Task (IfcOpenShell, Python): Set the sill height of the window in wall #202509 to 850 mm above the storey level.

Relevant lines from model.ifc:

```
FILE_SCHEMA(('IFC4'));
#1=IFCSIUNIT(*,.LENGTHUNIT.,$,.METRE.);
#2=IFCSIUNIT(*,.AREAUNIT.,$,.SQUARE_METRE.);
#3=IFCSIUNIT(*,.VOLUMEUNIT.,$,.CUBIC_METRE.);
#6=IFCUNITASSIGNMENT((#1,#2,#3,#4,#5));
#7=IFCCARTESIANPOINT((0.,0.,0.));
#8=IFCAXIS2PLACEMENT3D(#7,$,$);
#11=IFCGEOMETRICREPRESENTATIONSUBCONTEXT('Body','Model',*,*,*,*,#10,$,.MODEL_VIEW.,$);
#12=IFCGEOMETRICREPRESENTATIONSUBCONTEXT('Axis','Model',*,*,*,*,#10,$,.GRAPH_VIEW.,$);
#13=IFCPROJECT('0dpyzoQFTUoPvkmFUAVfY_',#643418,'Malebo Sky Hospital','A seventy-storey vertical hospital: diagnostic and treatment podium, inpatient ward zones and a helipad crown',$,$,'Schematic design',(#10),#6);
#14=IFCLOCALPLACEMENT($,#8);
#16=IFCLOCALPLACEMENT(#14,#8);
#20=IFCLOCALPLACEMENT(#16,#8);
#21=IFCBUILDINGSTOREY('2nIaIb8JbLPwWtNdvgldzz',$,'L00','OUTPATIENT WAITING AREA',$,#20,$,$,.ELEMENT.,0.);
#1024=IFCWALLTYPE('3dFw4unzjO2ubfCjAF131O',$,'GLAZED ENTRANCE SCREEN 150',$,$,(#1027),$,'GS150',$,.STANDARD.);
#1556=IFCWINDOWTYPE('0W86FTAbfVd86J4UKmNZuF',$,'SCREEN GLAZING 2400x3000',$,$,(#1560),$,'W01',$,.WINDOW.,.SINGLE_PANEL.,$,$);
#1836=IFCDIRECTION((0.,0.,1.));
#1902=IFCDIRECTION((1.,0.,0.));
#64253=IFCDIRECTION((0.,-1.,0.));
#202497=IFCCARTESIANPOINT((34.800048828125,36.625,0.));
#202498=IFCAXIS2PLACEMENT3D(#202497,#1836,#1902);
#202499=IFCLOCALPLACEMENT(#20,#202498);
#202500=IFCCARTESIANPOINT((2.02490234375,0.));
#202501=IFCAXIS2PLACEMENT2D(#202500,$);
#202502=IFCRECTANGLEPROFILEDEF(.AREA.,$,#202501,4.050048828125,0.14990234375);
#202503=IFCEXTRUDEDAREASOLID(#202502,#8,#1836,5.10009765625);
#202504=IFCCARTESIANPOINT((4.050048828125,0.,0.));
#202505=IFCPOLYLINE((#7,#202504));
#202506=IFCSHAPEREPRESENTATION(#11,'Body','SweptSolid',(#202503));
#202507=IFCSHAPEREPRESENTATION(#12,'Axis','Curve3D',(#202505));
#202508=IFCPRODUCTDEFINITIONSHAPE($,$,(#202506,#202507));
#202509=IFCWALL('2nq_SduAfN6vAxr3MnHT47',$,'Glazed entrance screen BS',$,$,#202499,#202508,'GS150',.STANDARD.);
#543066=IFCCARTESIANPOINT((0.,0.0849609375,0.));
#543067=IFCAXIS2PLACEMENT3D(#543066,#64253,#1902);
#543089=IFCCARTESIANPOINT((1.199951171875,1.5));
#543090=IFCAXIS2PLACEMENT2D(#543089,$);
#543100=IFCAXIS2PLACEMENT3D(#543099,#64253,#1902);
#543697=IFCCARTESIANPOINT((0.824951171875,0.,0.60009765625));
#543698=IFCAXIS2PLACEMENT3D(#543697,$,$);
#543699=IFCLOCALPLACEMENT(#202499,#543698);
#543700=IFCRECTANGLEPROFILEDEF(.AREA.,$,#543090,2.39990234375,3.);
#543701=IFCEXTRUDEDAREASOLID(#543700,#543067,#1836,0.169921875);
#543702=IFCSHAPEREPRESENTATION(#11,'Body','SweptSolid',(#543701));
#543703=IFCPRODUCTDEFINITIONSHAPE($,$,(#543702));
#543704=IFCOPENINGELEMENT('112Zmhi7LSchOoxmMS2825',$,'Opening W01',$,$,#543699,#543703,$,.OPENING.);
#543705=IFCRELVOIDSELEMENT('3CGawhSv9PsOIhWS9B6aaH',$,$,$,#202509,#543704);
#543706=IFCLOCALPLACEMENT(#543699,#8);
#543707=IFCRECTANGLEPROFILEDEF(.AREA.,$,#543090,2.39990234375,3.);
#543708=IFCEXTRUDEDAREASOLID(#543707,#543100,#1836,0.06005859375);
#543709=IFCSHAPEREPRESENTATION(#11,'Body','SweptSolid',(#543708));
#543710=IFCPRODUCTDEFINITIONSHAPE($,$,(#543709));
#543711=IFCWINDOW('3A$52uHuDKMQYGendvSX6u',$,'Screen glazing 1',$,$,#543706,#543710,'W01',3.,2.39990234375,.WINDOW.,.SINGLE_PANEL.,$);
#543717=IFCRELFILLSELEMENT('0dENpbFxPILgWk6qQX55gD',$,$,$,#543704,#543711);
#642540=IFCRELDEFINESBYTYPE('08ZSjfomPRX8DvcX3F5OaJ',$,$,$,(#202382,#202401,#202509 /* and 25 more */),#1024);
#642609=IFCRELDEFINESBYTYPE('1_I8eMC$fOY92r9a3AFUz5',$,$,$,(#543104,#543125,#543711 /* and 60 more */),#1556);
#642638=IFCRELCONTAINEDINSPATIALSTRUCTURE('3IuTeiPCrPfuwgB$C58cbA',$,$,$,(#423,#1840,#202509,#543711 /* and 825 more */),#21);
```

```python
import numpy as np
import ifcopenshell
import ifcopenshell.api.geometry
import ifcopenshell.geom
import ifcopenshell.util.element
import ifcopenshell.util.placement
import ifcopenshell.util.shape
import ifcopenshell.util.unit

model = ifcopenshell.open("model.ifc")
unit_scale = ifcopenshell.util.unit.calculate_unit_scale(model)

window = model.by_guid("3A$52uHuDKMQYGendvSX6u")
opening = window.FillsVoids[0].RelatingOpeningElement
storey = ifcopenshell.util.element.get_container(window, ifc_class="IfcBuildingStorey")
level = ifcopenshell.util.placement.get_local_placement(storey.ObjectPlacement)[2, 3]

# The opening's origin need not be at the sill, so measure its lowest point.
shape = ifcopenshell.geom.create_shape(ifcopenshell.geom.settings(), opening)
bottom = ifcopenshell.util.shape.get_shape_bottom_elevation(shape, shape.geometry) / unit_scale
dz = level + 0.85 - bottom

shift = np.array([0.0, 0.0, dz])
# The window is placed relative to its opening, so it follows when the opening moves.
matrix = ifcopenshell.util.placement.get_local_placement(opening.ObjectPlacement)
matrix[:3, 3] += shift
ifcopenshell.api.geometry.edit_object_placement(
    model, product=opening, matrix=matrix, is_si=False, should_transform_children=True
)

print(f"moved by {dz * unit_scale:+.3f} m")

model.write("model_updated.ifc")
```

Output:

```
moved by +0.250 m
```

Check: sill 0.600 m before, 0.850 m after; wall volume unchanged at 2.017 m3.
